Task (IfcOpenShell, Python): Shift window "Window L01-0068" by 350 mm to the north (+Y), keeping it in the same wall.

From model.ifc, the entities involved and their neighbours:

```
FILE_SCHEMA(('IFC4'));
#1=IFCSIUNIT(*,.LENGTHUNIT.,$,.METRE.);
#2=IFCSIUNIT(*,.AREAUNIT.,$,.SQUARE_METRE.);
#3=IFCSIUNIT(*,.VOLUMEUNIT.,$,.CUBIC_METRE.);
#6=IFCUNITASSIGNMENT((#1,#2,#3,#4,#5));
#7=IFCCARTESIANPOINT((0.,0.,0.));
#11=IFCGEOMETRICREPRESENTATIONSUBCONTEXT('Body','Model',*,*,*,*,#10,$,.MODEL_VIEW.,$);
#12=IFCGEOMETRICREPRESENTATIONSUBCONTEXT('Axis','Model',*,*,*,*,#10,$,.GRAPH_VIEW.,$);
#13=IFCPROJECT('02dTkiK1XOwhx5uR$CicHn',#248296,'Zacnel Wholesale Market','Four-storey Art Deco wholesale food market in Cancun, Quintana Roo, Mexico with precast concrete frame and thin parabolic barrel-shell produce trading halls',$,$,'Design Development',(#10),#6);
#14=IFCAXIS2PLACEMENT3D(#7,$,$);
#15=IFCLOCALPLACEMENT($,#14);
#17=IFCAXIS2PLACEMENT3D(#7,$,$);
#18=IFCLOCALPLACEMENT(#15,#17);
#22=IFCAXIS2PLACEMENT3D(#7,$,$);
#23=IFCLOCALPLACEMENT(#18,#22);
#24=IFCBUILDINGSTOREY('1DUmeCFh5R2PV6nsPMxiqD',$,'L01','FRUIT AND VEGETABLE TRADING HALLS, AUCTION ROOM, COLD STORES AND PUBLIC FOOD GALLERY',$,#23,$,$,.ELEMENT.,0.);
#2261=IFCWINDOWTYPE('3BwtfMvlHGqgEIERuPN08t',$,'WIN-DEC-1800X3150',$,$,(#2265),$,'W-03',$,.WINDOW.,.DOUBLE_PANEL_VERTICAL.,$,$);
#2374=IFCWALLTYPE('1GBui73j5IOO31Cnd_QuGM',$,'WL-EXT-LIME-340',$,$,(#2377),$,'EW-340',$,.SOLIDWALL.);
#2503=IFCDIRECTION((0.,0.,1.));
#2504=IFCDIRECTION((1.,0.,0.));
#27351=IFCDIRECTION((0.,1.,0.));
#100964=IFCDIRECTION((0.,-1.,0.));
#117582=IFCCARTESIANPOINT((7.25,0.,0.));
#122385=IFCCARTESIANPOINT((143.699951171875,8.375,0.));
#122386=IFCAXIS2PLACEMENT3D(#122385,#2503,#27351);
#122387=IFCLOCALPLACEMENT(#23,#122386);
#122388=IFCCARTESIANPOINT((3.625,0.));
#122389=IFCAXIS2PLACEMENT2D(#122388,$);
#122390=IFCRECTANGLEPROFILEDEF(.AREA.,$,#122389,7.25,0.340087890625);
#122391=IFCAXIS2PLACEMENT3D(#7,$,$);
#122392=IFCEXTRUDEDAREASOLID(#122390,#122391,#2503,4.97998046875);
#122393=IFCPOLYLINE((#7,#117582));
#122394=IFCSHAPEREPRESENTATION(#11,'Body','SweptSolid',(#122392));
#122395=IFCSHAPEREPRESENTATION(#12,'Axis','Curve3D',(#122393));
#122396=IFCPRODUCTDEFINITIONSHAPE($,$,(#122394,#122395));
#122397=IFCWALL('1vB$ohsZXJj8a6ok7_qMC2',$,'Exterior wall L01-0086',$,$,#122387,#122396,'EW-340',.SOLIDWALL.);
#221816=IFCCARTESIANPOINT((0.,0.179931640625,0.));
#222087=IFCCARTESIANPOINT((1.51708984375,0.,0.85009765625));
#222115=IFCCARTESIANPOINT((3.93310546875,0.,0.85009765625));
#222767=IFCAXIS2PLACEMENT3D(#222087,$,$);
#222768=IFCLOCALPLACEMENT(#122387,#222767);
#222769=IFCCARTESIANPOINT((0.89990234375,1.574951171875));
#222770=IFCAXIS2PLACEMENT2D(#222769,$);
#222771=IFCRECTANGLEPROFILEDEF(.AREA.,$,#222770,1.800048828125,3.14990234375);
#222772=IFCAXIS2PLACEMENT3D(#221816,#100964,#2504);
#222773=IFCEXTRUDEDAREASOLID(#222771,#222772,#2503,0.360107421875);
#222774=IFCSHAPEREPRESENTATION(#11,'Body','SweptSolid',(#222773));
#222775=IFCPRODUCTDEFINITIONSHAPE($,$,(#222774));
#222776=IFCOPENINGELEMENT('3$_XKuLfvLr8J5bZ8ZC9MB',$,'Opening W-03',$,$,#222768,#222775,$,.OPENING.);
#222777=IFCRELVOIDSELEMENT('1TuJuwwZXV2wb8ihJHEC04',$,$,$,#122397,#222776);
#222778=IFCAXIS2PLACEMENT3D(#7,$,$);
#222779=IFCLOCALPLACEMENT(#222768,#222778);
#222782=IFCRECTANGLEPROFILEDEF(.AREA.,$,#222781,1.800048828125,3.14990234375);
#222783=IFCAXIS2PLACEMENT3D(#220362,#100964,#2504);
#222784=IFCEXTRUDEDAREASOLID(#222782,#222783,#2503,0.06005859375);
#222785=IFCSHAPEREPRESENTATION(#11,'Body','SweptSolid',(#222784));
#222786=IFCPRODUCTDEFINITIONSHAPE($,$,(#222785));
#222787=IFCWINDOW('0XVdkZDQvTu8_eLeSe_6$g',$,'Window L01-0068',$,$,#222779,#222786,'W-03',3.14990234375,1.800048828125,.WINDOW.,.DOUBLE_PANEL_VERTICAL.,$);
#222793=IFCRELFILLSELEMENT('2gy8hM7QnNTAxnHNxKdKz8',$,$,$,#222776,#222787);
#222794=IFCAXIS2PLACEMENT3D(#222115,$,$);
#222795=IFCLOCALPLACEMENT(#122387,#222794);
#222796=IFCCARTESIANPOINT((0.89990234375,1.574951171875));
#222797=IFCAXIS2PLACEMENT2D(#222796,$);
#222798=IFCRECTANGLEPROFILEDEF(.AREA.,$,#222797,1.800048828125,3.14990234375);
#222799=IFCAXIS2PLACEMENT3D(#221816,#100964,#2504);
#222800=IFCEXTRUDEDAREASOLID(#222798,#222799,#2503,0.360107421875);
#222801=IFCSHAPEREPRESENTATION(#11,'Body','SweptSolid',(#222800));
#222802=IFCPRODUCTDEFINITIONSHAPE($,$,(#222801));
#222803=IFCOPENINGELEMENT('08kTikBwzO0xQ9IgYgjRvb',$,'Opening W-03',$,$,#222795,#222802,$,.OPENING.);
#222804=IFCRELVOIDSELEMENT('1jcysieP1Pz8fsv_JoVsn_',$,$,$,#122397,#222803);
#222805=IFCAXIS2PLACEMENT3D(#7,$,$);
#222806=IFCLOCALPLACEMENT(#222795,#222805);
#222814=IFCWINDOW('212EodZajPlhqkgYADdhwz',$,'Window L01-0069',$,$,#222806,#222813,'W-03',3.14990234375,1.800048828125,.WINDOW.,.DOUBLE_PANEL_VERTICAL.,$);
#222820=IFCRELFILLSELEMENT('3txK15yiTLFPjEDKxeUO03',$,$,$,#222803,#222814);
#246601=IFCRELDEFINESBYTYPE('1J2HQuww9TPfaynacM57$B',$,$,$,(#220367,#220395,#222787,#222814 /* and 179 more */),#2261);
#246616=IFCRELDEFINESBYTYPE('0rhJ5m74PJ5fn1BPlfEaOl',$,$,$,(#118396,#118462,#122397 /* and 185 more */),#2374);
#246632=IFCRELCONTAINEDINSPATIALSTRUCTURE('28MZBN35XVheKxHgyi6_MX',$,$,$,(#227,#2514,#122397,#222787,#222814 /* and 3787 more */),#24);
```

```python
import ifcopenshell
import ifcopenshell.api.geometry
import ifcopenshell.util.placement
import ifcopenshell.util.unit

model = ifcopenshell.open("model.ifc")
unit_scale = ifcopenshell.util.unit.calculate_unit_scale(model)

window = model.by_guid("0XVdkZDQvTu8_eLeSe_6$g")
opening = window.FillsVoids[0].RelatingOpeningElement
wall = opening.VoidsElements[0].RelatingBuildingElement

wall_matrix = ifcopenshell.util.placement.get_local_placement(wall.ObjectPlacement)
shift = wall_matrix[:3, 0] * 0.35 / unit_scale
before = ifcopenshell.util.placement.get_local_placement(window.ObjectPlacement)[:3, 3].copy()

# The window is placed relative to its opening, so it follows when the opening moves.
matrix = ifcopenshell.util.placement.get_local_placement(opening.ObjectPlacement)
matrix[:3, 3] += shift
ifcopenshell.api.geometry.edit_object_placement(
    model, product=opening, matrix=matrix, is_si=False, should_transform_children=True
)

after = ifcopenshell.util.placement.get_local_placement(window.ObjectPlacement)[:3, 3]
print("window moved by", (after - before).round(3) + 0.0)

model.write("model_updated.ifc")
```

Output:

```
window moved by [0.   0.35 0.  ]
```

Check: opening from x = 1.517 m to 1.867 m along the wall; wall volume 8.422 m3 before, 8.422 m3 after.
